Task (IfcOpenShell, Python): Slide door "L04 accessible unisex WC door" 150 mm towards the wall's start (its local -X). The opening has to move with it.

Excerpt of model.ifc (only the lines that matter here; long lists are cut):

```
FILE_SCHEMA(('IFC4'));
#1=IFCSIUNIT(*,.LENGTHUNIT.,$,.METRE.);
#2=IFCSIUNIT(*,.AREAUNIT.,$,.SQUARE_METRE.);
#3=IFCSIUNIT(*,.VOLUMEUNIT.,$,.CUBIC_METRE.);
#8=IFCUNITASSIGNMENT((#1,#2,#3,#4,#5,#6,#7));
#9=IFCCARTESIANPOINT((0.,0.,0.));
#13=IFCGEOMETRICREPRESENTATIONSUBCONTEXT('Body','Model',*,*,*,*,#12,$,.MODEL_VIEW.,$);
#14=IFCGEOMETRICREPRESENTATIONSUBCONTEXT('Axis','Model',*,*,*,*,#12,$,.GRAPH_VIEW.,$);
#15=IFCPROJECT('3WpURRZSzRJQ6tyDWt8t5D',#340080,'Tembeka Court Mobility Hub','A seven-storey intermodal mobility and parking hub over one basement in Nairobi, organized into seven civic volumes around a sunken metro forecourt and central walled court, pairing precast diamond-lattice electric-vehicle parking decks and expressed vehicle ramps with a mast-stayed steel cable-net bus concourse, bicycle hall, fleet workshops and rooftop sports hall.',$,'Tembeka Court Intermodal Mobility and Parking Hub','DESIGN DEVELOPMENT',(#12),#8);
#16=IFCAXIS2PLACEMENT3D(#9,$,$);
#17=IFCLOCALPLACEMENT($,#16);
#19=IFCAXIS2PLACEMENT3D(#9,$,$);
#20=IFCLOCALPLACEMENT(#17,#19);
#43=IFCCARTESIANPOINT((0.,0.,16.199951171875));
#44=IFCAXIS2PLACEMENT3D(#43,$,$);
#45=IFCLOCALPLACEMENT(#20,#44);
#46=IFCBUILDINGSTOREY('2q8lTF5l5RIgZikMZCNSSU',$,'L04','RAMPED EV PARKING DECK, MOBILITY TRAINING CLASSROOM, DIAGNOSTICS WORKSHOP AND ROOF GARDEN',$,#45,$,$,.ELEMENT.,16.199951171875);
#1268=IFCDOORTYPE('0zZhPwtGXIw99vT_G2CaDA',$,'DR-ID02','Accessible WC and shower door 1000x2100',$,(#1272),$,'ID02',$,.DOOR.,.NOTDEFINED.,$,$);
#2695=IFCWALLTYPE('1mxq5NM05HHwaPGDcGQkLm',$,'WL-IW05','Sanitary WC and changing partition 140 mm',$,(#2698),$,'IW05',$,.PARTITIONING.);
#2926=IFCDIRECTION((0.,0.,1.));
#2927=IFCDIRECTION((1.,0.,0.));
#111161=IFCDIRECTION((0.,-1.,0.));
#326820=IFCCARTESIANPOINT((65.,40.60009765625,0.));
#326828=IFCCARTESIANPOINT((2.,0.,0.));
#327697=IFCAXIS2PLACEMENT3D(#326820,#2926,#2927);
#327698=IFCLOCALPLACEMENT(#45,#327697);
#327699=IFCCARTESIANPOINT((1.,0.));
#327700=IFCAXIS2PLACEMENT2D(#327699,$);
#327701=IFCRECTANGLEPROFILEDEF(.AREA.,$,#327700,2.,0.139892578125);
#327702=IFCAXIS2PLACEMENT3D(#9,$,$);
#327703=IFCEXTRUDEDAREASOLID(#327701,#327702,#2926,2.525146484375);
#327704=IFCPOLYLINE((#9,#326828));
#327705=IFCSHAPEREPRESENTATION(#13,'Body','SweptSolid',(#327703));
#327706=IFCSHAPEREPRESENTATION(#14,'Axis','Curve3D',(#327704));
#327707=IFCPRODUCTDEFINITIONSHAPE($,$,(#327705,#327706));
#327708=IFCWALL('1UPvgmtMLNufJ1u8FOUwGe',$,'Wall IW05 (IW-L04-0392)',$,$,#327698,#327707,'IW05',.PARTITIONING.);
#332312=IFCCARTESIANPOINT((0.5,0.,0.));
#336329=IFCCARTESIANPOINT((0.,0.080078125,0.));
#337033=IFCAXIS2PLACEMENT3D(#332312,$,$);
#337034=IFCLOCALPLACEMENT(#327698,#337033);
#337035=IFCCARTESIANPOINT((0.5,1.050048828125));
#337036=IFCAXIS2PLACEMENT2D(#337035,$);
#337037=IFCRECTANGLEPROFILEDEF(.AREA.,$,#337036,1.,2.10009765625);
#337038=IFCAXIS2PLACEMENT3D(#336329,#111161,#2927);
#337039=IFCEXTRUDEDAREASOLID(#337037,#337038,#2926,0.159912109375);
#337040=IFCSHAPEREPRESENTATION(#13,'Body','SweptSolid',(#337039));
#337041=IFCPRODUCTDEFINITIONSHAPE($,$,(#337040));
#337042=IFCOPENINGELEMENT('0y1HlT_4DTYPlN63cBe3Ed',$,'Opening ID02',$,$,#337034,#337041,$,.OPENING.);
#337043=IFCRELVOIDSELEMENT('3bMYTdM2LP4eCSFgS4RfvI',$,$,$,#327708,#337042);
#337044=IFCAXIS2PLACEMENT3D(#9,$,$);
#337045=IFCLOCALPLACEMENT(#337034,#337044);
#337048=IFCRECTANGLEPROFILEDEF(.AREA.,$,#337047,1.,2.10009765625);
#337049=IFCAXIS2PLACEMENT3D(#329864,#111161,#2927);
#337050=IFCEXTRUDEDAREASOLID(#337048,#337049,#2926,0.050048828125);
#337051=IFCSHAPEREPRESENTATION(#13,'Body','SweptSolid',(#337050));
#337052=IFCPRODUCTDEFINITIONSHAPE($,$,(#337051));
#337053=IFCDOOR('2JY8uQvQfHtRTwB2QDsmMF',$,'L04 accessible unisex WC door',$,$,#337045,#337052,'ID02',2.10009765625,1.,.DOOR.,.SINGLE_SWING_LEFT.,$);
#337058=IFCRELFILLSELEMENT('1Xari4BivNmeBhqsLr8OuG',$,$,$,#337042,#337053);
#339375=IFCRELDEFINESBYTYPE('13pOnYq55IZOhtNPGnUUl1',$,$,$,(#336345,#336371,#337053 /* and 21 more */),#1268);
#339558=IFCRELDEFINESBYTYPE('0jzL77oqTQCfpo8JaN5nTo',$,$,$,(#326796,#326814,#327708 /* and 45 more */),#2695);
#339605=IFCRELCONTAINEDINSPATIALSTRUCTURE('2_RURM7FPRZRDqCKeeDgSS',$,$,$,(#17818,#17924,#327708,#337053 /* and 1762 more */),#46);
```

```python
import ifcopenshell
import ifcopenshell.api.geometry
import ifcopenshell.util.placement
import ifcopenshell.util.unit

model = ifcopenshell.open("model.ifc")
unit_scale = ifcopenshell.util.unit.calculate_unit_scale(model)

door = model.by_guid("2JY8uQvQfHtRTwB2QDsmMF")
opening = door.FillsVoids[0].RelatingOpeningElement
wall = opening.VoidsElements[0].RelatingBuildingElement

wall_matrix = ifcopenshell.util.placement.get_local_placement(wall.ObjectPlacement)
shift = wall_matrix[:3, 0] * -0.15 / unit_scale
before = ifcopenshell.util.placement.get_local_placement(door.ObjectPlacement)[:3, 3].copy()

# The door is placed relative to its opening, so it follows when the opening moves.
matrix = ifcopenshell.util.placement.get_local_placement(opening.ObjectPlacement)
matrix[:3, 3] += shift
ifcopenshell.api.geometry.edit_object_placement(
    model, product=opening, matrix=matrix, is_si=False, should_transform_children=True
)

after = ifcopenshell.util.placement.get_local_placement(door.ObjectPlacement)[:3, 3]
print("door moved by", (after - before).round(3) + 0.0)

model.write("model_updated.ifc")
```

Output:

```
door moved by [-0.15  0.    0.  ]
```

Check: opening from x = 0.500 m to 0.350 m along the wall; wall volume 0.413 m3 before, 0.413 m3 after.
